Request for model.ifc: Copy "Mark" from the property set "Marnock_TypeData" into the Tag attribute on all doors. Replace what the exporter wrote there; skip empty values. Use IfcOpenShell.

First a look at what the model holds.

```python
import ifcopenshell
import ifcopenshell.util.element

model = ifcopenshell.open("model.ifc")
print(model.schema)
doors = model.by_type("IfcDoor")
print(len(doors), "doors")
for e in doors[:8]:
    source = ifcopenshell.util.element.get_pset(e, "Marnock_TypeData", "Mark")
    target = e.Tag
    print(e.id(), repr(source), repr(target), sep=" | ")
```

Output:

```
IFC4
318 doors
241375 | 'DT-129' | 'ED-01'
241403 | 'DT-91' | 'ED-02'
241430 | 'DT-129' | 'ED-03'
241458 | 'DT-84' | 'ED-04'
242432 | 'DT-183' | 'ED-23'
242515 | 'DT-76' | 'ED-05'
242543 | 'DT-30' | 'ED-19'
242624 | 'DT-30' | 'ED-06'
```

```python
import ifcopenshell
import ifcopenshell.util.element

model = ifcopenshell.open("model.ifc")

count = 0
for e in model.by_type("IfcDoor"):
    value = ifcopenshell.util.element.get_pset(e, "Marnock_TypeData", "Mark")
    current = e.Tag
    if not value or not value.strip() or current == value:
        continue
    e.Tag = value
    count += 1

print(count, "doors updated")

model.write("model-out.ifc")
```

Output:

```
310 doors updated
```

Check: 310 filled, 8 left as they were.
